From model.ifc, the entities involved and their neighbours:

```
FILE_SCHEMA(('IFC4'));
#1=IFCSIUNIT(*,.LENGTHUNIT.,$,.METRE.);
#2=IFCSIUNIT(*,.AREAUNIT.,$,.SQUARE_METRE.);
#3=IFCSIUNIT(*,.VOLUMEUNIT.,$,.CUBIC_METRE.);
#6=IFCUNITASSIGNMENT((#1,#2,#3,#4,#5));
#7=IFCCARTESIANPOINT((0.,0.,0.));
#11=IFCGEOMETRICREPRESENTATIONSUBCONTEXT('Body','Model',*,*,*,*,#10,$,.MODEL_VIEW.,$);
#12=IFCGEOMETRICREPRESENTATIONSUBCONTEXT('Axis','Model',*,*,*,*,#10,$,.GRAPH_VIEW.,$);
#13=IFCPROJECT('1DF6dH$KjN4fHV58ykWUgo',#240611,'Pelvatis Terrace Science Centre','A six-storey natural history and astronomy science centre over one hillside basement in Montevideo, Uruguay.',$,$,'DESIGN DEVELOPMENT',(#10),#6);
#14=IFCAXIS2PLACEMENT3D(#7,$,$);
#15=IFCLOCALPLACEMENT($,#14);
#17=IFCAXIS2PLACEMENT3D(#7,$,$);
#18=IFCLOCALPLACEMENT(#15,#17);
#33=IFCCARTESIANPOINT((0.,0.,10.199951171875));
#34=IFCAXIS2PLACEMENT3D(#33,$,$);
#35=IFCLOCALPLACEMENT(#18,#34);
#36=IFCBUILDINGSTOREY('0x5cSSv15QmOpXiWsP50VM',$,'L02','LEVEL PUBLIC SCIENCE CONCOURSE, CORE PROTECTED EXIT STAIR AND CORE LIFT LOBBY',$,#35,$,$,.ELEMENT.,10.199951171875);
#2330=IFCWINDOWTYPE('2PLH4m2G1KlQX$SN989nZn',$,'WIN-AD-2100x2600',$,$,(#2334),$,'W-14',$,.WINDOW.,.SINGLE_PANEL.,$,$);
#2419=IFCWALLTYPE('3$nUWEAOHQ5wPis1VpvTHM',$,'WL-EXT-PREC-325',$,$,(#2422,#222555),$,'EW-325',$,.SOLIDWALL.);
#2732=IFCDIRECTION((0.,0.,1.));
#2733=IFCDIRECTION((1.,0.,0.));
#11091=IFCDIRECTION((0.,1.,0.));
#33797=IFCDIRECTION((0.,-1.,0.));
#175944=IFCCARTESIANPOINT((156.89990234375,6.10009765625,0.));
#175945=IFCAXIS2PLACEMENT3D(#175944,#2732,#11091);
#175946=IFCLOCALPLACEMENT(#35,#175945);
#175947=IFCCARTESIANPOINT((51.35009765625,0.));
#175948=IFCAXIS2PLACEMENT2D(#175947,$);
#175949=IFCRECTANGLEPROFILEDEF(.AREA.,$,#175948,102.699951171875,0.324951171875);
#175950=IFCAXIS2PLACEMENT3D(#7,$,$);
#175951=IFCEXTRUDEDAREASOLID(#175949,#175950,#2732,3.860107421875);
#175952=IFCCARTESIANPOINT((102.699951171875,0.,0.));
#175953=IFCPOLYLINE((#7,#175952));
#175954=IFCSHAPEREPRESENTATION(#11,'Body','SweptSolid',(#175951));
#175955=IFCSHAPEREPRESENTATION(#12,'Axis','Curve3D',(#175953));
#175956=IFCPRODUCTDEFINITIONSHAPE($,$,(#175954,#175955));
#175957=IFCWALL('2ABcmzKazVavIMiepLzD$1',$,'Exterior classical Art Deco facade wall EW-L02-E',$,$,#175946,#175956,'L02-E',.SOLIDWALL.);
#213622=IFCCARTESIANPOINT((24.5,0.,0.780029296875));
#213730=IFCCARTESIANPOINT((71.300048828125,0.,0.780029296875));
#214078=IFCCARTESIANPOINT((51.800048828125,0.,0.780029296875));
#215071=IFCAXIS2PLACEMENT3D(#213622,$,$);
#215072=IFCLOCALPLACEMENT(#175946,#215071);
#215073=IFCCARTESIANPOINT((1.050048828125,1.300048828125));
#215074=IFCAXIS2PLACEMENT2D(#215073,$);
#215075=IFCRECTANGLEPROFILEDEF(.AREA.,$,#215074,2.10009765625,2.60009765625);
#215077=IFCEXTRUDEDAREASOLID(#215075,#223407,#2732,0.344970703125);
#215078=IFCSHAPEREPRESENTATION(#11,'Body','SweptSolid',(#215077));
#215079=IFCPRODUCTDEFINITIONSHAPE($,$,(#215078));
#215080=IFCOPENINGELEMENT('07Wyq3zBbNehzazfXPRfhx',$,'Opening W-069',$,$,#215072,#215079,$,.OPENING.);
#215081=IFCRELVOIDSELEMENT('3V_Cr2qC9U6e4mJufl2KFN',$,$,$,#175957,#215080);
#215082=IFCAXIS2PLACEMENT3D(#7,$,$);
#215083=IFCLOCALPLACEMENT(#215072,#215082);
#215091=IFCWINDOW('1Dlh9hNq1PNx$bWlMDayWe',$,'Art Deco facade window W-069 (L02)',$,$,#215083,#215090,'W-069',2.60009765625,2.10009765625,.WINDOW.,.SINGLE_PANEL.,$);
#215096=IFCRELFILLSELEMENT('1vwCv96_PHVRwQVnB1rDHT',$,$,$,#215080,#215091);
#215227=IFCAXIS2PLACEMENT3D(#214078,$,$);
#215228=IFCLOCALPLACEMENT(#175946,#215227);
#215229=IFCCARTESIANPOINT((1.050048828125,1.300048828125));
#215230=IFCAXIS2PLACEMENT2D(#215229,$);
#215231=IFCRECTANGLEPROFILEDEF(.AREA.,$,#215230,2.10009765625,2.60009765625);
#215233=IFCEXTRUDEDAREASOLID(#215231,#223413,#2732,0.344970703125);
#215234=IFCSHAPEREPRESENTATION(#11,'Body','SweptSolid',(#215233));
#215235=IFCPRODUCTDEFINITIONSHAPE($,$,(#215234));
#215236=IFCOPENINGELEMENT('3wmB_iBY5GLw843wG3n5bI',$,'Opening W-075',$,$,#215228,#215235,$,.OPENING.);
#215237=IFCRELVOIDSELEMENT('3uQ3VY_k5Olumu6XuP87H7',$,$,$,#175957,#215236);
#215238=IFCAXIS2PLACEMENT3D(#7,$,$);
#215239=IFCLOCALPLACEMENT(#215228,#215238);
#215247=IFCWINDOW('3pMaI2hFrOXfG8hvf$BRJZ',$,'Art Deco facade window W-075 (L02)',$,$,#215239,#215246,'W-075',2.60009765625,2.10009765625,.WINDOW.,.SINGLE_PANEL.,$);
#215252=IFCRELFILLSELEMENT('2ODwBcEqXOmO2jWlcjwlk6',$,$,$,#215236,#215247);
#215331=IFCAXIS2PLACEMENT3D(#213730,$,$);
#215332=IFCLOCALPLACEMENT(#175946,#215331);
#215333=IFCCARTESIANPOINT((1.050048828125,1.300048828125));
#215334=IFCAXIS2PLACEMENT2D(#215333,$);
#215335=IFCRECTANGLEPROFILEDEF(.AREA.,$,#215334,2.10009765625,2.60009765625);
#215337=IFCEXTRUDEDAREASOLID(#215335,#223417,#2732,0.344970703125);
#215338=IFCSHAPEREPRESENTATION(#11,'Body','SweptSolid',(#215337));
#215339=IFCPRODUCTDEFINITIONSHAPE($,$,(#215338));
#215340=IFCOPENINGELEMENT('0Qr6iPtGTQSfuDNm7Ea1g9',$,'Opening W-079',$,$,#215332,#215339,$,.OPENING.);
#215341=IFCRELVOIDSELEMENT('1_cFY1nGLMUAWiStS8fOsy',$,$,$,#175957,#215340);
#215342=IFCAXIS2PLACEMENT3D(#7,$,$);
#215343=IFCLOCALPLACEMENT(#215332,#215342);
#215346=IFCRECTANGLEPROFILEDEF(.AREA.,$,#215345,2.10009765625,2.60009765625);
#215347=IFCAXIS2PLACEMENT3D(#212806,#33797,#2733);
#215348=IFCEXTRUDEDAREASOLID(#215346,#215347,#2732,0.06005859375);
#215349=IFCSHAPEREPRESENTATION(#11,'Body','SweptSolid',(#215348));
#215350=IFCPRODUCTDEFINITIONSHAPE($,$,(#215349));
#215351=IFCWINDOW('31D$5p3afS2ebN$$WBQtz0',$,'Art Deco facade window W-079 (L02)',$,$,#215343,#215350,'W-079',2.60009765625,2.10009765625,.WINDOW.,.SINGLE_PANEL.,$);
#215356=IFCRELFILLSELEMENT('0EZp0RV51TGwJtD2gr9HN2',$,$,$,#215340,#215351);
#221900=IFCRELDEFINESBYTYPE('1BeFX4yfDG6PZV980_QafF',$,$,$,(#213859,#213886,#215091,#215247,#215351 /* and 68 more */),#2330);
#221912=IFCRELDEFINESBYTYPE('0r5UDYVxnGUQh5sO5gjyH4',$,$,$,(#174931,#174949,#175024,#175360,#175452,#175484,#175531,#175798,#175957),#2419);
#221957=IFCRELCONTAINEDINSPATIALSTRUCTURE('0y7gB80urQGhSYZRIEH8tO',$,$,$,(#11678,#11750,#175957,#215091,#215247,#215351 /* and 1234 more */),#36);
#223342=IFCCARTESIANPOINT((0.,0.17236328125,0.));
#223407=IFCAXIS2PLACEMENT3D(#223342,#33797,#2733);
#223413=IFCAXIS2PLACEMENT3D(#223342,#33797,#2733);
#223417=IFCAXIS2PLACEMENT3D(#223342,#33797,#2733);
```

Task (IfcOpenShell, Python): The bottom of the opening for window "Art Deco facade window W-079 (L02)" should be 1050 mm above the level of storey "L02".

```python
import numpy as np
import ifcopenshell
import ifcopenshell.api.geometry
import ifcopenshell.geom
import ifcopenshell.util.element
import ifcopenshell.util.placement
import ifcopenshell.util.shape
import ifcopenshell.util.unit

model = ifcopenshell.open("model.ifc")
unit_scale = ifcopenshell.util.unit.calculate_unit_scale(model)

window = model.by_id(215351)
opening = window.FillsVoids[0].RelatingOpeningElement
storey = ifcopenshell.util.element.get_container(window, ifc_class="IfcBuildingStorey")
level = ifcopenshell.util.placement.get_local_placement(storey.ObjectPlacement)[2, 3]

# The opening's origin need not be at the sill, so measure its lowest point.
shape = ifcopenshell.geom.create_shape(ifcopenshell.geom.settings(), opening)
bottom = ifcopenshell.util.shape.get_shape_bottom_elevation(shape, shape.geometry) / unit_scale
dz = level + 1.05 - bottom

shift = np.array([0.0, 0.0, dz])
# The window is placed relative to its opening, so it follows when the opening moves.
matrix = ifcopenshell.util.placement.get_local_placement(opening.ObjectPlacement)
matrix[:3, 3] += shift
ifcopenshell.api.geometry.edit_object_placement(
    model, product=opening, matrix=matrix, is_si=False, should_transform_children=True
)

print(f"moved by {dz * unit_scale:+.3f} m")

model.write("model_edited.ifc")
```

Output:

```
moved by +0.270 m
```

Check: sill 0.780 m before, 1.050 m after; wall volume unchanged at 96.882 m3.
